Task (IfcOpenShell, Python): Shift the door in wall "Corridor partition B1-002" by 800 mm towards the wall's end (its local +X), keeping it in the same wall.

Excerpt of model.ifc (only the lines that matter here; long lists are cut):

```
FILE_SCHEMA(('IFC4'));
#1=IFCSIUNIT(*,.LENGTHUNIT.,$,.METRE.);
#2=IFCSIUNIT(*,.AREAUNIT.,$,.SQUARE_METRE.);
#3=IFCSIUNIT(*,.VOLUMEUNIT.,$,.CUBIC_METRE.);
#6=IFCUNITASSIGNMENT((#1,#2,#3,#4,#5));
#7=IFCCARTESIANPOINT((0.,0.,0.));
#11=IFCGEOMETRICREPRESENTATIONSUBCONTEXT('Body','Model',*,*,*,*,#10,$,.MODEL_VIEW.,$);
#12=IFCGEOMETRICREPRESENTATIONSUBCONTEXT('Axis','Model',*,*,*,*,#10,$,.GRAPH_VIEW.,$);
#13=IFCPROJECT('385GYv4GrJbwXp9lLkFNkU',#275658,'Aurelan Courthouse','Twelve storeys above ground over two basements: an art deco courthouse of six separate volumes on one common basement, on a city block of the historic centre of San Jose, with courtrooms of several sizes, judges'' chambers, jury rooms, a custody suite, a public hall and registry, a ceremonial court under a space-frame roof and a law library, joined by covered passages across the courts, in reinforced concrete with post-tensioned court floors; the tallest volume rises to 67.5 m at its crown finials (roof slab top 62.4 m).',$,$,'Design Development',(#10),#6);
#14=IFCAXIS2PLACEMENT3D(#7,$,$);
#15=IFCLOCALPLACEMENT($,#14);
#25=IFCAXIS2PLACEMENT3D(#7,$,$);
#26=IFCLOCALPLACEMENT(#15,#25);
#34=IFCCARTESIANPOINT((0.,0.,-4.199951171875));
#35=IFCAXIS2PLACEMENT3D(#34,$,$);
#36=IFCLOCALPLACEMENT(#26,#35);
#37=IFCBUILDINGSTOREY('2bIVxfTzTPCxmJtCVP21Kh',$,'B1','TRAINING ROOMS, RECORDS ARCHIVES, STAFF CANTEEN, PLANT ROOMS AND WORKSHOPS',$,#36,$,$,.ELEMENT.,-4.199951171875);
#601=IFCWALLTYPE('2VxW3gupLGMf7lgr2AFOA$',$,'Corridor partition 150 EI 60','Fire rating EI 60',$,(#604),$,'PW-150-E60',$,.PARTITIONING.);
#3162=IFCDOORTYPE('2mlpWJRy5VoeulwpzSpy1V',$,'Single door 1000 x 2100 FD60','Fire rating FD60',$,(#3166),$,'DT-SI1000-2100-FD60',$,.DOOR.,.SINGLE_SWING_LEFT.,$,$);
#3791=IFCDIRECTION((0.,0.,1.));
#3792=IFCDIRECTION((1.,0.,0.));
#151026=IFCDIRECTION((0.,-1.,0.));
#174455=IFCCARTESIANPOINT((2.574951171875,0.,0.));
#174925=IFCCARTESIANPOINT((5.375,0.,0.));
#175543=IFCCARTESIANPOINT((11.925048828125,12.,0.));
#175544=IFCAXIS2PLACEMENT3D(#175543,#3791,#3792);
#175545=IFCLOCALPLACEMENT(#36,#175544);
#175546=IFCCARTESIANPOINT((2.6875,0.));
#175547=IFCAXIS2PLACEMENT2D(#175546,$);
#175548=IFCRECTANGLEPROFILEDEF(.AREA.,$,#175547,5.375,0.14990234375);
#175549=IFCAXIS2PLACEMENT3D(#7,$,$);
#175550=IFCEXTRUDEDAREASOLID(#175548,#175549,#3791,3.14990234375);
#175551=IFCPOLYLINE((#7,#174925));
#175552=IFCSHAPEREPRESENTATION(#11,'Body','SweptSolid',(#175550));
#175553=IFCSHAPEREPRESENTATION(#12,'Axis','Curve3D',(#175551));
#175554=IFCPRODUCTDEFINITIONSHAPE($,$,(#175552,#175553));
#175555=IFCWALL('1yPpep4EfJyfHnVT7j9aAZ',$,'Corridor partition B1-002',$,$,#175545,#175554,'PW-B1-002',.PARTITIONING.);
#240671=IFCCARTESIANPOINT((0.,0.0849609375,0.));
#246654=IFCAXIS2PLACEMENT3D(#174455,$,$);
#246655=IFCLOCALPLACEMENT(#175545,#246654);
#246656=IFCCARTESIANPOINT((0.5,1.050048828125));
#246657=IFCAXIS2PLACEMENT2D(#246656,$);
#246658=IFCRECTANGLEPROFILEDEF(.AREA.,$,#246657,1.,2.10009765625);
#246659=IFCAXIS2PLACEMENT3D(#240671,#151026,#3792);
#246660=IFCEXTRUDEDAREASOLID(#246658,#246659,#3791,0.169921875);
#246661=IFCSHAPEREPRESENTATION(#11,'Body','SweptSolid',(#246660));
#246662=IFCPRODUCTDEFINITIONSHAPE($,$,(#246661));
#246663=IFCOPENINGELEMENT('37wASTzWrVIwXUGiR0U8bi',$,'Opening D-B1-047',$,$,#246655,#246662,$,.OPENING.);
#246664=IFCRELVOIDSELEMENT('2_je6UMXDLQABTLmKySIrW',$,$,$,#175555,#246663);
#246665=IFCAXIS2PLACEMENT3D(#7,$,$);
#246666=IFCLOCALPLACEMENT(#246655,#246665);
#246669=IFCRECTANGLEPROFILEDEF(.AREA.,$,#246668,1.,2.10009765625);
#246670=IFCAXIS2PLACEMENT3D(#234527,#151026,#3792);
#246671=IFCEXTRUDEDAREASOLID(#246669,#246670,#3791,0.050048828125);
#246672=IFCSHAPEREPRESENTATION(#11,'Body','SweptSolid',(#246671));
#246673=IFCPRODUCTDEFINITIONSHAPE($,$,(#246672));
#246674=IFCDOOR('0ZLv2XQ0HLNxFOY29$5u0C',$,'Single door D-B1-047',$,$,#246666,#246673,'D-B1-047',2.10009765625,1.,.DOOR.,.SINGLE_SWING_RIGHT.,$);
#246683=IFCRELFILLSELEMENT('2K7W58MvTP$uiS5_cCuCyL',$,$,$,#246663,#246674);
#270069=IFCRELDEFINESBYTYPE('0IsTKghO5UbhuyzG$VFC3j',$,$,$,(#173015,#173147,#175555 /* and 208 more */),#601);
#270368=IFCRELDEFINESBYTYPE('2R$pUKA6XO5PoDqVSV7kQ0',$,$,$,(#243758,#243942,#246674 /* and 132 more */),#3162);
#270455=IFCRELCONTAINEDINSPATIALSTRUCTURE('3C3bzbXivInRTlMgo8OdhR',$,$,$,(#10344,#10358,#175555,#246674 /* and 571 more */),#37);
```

```python
import ifcopenshell
import ifcopenshell.api.geometry
import ifcopenshell.util.placement
import ifcopenshell.util.unit

model = ifcopenshell.open("model.ifc")
unit_scale = ifcopenshell.util.unit.calculate_unit_scale(model)

door = model.by_guid("0ZLv2XQ0HLNxFOY29$5u0C")
opening = door.FillsVoids[0].RelatingOpeningElement
wall = opening.VoidsElements[0].RelatingBuildingElement

wall_matrix = ifcopenshell.util.placement.get_local_placement(wall.ObjectPlacement)
shift = wall_matrix[:3, 0] * 0.8 / unit_scale
before = ifcopenshell.util.placement.get_local_placement(door.ObjectPlacement)[:3, 3].copy()

# The door is placed relative to its opening, so it follows when the opening moves.
matrix = ifcopenshell.util.placement.get_local_placement(opening.ObjectPlacement)
matrix[:3, 3] += shift
ifcopenshell.api.geometry.edit_object_placement(
    model, product=opening, matrix=matrix, is_si=False, should_transform_children=True
)

after = ifcopenshell.util.placement.get_local_placement(door.ObjectPlacement)[:3, 3]
print("door moved by", (after - before).round(3) + 0.0)

model.write("model_rev.ifc")
```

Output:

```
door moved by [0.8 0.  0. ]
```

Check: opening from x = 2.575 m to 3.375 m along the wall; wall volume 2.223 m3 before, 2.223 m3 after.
